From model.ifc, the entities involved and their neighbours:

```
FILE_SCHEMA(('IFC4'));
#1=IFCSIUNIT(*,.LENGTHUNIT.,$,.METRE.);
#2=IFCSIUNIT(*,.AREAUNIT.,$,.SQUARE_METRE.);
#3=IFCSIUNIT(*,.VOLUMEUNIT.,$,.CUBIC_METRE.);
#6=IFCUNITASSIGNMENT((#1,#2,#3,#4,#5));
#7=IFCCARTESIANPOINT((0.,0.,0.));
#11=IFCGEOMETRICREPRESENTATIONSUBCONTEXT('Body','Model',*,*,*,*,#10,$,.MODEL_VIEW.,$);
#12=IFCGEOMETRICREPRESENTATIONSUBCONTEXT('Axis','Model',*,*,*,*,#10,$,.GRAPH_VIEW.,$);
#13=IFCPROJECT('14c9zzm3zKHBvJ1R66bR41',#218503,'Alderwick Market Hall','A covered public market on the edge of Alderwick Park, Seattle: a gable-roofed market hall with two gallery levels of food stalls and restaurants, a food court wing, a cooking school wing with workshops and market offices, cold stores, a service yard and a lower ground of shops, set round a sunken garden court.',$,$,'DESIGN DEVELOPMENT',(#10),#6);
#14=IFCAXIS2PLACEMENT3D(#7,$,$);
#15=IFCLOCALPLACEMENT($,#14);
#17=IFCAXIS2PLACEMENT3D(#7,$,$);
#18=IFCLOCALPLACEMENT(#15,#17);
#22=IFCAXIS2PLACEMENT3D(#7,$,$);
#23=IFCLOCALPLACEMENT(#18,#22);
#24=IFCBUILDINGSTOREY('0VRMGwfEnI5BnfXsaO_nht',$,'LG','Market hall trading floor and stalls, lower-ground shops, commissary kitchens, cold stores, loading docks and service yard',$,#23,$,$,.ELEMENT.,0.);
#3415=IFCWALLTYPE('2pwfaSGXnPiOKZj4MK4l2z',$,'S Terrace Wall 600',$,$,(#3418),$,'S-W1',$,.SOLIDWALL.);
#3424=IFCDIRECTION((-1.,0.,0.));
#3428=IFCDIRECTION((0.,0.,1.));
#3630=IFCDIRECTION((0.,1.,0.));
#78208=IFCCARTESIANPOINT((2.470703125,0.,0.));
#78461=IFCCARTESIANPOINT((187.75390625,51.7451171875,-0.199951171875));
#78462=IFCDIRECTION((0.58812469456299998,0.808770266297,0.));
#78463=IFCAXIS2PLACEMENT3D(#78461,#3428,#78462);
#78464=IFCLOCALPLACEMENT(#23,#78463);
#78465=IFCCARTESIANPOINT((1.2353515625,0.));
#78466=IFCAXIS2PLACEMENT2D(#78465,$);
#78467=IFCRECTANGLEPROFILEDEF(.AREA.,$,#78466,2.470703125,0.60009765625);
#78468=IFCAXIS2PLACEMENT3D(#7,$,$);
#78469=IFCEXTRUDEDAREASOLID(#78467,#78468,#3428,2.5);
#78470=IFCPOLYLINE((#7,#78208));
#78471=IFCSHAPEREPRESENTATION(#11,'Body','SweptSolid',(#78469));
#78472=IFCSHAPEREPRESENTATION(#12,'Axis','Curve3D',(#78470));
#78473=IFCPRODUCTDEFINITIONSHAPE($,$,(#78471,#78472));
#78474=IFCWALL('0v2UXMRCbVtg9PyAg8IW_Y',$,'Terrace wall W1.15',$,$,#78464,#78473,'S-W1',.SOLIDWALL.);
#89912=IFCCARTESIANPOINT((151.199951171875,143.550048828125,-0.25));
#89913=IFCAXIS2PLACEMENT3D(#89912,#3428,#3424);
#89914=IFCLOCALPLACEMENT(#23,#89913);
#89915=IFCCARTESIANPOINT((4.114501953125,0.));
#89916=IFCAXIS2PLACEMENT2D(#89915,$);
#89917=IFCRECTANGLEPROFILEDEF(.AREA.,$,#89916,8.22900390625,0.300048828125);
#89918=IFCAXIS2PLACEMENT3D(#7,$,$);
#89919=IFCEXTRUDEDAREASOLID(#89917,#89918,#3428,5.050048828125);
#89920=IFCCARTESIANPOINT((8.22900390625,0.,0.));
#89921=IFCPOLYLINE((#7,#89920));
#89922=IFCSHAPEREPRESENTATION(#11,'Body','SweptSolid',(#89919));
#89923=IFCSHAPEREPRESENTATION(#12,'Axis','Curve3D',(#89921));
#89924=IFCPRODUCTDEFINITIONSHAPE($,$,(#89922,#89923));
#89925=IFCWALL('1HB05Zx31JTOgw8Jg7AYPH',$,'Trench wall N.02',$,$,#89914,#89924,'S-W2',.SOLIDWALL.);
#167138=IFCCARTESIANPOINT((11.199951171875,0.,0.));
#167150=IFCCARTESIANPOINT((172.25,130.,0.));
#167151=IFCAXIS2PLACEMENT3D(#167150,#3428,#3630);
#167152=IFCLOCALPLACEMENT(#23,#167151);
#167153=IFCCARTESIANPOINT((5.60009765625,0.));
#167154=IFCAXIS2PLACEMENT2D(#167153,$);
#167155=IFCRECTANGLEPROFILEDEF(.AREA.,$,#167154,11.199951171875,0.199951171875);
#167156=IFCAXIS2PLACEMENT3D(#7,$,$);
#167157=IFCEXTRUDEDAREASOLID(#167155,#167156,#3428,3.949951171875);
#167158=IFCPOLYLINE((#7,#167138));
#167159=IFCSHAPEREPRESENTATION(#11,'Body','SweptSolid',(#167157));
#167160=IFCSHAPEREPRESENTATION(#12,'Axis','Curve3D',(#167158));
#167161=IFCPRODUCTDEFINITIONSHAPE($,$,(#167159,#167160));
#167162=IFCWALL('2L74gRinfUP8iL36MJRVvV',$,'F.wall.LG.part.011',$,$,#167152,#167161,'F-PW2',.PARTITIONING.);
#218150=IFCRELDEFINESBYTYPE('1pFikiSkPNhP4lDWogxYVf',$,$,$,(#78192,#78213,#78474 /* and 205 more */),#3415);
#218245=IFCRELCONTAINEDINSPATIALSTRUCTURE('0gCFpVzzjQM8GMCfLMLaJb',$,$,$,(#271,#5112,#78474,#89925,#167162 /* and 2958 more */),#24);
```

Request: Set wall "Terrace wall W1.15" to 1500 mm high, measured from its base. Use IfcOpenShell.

```python
import ifcopenshell
import ifcopenshell.geom
import ifcopenshell.util.representation
import ifcopenshell.util.shape
import ifcopenshell.util.unit

model = ifcopenshell.open("model.ifc")
unit_scale = ifcopenshell.util.unit.calculate_unit_scale(model)
settings = ifcopenshell.geom.settings()


def volume(element):
    """Net volume in cubic metres, openings subtracted."""
    shape = ifcopenshell.geom.create_shape(settings, element)
    return ifcopenshell.util.shape.get_volume(shape.geometry)


wall = model.by_guid("0v2UXMRCbVtg9PyAg8IW_Y")
before = volume(wall)

body = ifcopenshell.util.representation.get_representation(wall, "Model", "Body")
solid = body.Items[0]
old_height = solid.Depth
solid.Depth = 1.5 / unit_scale
after = volume(wall)

print(f"height {old_height:g} -> {solid.Depth:g}, volume {before:.3f} -> {after:.3f} m3")

model.write("model_v2.ifc")
```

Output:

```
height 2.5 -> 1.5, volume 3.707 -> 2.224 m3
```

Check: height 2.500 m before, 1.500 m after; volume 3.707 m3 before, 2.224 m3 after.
